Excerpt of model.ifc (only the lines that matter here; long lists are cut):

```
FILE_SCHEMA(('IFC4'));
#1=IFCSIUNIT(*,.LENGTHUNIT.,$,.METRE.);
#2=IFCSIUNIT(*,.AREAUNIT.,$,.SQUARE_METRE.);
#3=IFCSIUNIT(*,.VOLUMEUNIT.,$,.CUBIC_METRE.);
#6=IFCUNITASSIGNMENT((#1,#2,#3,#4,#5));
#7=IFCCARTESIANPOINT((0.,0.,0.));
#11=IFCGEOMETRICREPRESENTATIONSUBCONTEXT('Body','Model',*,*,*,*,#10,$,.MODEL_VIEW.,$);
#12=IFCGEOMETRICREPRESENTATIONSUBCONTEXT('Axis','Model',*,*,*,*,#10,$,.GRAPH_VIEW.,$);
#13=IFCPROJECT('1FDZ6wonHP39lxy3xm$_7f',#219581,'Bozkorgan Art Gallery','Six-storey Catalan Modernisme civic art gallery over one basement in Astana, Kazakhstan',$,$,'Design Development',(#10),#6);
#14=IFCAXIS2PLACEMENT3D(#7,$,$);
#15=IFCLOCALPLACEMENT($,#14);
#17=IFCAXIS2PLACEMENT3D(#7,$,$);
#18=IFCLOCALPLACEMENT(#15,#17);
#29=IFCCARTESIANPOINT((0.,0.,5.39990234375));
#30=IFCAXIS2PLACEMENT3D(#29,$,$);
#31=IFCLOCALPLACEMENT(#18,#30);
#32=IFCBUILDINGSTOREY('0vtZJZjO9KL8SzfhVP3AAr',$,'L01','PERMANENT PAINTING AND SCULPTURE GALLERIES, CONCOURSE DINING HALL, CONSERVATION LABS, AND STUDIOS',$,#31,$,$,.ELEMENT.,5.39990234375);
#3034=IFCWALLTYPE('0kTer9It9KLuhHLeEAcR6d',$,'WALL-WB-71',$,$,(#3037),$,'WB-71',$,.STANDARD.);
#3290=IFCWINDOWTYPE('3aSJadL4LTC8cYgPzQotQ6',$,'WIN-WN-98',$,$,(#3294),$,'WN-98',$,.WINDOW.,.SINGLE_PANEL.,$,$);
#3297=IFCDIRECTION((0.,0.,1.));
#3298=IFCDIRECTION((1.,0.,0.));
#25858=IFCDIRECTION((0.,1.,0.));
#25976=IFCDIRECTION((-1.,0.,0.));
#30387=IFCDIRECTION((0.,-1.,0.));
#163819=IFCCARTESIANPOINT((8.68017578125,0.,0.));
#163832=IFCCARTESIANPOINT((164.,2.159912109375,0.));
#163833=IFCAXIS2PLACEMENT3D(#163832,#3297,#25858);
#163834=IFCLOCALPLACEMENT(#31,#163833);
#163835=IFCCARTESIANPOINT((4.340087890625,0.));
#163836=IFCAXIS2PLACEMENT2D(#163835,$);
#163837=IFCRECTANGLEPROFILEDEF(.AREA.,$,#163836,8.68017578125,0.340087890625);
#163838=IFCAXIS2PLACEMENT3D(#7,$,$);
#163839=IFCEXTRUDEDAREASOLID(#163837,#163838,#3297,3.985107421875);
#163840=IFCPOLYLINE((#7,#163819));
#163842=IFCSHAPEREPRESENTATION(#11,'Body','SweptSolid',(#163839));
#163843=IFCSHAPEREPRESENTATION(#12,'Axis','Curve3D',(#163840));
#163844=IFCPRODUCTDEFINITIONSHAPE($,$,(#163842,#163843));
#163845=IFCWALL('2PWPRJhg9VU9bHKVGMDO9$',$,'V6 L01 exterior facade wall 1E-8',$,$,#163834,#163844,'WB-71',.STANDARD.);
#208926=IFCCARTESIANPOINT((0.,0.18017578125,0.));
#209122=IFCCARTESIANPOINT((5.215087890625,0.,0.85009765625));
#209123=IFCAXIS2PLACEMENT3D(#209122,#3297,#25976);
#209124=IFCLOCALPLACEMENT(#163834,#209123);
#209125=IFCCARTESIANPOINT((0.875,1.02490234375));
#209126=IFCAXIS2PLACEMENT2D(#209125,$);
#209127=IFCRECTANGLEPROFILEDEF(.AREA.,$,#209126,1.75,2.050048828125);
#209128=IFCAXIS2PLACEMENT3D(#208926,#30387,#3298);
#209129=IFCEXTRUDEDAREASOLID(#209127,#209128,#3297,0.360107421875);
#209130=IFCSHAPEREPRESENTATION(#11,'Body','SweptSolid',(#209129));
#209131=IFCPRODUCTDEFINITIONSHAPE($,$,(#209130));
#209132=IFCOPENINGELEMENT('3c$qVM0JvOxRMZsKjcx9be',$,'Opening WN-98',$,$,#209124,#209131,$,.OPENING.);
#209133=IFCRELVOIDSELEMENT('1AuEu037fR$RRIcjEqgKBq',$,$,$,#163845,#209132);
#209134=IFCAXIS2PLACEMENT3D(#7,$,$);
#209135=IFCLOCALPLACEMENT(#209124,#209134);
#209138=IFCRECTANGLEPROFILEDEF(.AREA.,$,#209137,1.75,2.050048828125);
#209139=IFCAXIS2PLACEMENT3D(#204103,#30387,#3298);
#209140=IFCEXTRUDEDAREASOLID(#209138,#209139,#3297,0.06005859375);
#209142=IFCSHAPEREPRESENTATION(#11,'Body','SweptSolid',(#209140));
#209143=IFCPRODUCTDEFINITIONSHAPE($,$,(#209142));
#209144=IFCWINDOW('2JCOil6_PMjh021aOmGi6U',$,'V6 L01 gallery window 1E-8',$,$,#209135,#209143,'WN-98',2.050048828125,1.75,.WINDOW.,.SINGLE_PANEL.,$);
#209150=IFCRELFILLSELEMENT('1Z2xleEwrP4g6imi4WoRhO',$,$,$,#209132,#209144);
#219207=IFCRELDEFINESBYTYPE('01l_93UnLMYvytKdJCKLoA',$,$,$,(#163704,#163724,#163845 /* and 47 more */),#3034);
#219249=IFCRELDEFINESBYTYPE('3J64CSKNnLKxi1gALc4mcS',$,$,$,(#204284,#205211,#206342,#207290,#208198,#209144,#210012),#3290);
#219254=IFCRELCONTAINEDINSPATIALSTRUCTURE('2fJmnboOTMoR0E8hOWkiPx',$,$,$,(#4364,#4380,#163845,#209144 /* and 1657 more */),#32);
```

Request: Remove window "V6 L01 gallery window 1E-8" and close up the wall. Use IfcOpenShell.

```python
import ifcopenshell
import ifcopenshell.api.feature
import ifcopenshell.api.root
import ifcopenshell.geom
import ifcopenshell.util.shape

model = ifcopenshell.open("model.ifc")
settings = ifcopenshell.geom.settings()


def volume(element):
    """Net volume in cubic metres, openings subtracted."""
    shape = ifcopenshell.geom.create_shape(settings, element)
    return ifcopenshell.util.shape.get_volume(shape.geometry)


window = model.by_guid("2JCOil6_PMjh021aOmGi6U")
opening = window.FillsVoids[0].RelatingOpeningElement
wall = opening.VoidsElements[0].RelatingBuildingElement
before = volume(wall)

ifcopenshell.api.root.remove_product(model, product=window)
ifcopenshell.api.feature.remove_feature(model, feature=opening)

after = volume(wall)

print(f"wall volume {before:.3f} -> {after:.3f} m3")

model.write("model_updated.ifc")
```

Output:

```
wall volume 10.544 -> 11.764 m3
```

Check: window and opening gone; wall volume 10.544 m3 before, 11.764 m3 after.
